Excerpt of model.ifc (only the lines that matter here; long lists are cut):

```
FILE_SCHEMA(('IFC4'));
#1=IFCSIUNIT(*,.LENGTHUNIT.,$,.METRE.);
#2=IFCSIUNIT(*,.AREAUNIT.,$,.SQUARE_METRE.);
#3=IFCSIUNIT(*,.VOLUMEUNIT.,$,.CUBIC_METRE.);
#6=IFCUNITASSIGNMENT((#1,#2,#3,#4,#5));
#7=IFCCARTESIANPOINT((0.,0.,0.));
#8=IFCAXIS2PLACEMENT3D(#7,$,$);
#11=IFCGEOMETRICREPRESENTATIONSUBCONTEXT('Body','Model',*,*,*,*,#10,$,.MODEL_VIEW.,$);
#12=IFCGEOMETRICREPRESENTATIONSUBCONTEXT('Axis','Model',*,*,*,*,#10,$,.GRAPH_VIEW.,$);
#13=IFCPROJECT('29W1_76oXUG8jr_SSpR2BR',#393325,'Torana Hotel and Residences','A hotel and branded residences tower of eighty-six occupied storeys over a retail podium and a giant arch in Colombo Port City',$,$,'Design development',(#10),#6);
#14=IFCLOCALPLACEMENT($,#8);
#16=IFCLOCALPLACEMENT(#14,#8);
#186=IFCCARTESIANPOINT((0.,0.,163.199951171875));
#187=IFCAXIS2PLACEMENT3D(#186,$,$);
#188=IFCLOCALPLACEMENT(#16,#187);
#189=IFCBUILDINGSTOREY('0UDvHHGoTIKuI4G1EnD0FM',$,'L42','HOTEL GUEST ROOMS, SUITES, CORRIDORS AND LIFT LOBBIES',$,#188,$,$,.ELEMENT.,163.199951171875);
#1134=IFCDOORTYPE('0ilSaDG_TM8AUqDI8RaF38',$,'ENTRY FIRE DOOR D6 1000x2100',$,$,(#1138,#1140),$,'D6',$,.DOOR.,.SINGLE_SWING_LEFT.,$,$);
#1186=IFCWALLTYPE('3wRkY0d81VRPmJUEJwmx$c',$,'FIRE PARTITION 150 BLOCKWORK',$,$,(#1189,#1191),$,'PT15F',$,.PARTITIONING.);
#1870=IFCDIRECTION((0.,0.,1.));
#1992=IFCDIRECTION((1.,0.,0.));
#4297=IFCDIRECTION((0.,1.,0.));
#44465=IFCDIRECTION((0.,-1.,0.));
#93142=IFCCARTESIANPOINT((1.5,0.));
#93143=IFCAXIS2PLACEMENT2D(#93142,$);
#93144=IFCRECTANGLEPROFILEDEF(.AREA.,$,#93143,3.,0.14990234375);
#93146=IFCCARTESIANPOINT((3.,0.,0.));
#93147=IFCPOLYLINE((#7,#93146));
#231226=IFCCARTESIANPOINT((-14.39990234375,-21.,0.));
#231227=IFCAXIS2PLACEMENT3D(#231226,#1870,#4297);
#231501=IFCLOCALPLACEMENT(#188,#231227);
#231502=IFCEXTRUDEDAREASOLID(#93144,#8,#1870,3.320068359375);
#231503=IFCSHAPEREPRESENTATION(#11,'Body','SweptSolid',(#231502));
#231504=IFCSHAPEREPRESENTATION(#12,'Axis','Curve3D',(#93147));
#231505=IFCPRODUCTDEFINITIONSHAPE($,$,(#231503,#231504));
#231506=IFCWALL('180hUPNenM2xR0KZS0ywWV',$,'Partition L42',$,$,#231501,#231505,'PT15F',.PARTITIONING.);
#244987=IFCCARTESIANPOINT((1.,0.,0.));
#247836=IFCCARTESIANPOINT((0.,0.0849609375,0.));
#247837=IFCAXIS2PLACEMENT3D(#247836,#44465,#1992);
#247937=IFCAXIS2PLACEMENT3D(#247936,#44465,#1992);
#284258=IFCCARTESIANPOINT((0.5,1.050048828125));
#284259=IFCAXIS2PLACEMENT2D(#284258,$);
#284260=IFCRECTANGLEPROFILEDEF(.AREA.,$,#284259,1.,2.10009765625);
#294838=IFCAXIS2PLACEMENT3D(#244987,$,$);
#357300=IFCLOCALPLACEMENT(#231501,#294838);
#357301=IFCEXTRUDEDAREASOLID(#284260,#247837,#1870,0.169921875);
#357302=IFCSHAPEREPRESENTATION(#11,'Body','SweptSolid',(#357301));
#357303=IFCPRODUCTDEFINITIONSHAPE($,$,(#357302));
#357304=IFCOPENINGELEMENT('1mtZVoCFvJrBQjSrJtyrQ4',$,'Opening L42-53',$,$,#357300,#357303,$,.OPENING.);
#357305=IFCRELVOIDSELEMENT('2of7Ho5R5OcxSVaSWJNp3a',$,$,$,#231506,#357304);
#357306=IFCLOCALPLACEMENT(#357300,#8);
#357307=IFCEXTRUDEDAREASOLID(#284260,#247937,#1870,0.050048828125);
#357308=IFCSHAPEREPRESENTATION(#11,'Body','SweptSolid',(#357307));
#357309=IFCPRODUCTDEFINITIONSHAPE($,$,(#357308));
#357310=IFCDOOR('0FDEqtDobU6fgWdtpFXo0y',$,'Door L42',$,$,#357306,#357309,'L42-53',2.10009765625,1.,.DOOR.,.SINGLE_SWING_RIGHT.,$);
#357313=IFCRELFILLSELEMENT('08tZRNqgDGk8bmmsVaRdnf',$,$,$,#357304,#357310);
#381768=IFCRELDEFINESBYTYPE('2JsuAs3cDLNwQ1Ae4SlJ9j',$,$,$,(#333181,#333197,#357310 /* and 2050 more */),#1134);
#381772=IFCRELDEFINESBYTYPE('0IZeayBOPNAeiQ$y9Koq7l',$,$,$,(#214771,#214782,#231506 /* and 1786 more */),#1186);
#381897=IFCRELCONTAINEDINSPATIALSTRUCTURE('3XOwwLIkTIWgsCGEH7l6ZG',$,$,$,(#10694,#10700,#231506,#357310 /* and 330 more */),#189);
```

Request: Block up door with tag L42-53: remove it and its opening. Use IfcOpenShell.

```python
import ifcopenshell
import ifcopenshell.api.feature
import ifcopenshell.api.root
import ifcopenshell.geom
import ifcopenshell.util.shape

model = ifcopenshell.open("model.ifc")
settings = ifcopenshell.geom.settings()


def volume(element):
    """Net volume in cubic metres, openings subtracted."""
    shape = ifcopenshell.geom.create_shape(settings, element)
    return ifcopenshell.util.shape.get_volume(shape.geometry)


door = model.by_id(357310)
opening = door.FillsVoids[0].RelatingOpeningElement
wall = opening.VoidsElements[0].RelatingBuildingElement
before = volume(wall)

ifcopenshell.api.root.remove_product(model, product=door)
ifcopenshell.api.feature.remove_feature(model, feature=opening)

after = volume(wall)

print(f"wall volume {before:.3f} -> {after:.3f} m3")

model.write("model-out.ifc")
```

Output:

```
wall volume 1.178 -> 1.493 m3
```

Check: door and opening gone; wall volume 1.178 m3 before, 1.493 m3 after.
